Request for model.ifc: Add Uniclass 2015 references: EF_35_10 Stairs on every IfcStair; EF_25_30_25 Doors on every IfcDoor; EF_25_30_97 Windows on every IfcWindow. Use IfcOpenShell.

First a look at what the model holds.

```python
import ifcopenshell

model = ifcopenshell.open("model.ifc")
print(model.schema)
print("classifications:", [c.Name for c in model.by_type("IfcClassification")])
for ifc_class in ("IfcDoor", "IfcRoof", "IfcStair", "IfcWall", "IfcWindow"):
    print(ifc_class, len(model.by_type(ifc_class)))
```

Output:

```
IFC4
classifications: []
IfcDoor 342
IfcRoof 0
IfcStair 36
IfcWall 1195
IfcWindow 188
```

```python
import ifcopenshell
import ifcopenshell.api.classification

model = ifcopenshell.open("model.ifc")

system = ifcopenshell.api.classification.add_classification(model, classification="Uniclass 2015")

codes = {
    "IfcStair": ("EF_35_10", "Stairs"),
    "IfcDoor": ("EF_25_30_25", "Doors"),
    "IfcWindow": ("EF_25_30_97", "Windows"),
}
for ifc_class, (code, name) in codes.items():
    products = model.by_type(ifc_class)
    ifcopenshell.api.classification.add_reference(
        model, products=products, classification=system, identification=code, name=name
    )
    print(code, len(products))

model.write("model_updated.ifc")
```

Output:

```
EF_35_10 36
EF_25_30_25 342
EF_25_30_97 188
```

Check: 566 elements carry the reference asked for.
